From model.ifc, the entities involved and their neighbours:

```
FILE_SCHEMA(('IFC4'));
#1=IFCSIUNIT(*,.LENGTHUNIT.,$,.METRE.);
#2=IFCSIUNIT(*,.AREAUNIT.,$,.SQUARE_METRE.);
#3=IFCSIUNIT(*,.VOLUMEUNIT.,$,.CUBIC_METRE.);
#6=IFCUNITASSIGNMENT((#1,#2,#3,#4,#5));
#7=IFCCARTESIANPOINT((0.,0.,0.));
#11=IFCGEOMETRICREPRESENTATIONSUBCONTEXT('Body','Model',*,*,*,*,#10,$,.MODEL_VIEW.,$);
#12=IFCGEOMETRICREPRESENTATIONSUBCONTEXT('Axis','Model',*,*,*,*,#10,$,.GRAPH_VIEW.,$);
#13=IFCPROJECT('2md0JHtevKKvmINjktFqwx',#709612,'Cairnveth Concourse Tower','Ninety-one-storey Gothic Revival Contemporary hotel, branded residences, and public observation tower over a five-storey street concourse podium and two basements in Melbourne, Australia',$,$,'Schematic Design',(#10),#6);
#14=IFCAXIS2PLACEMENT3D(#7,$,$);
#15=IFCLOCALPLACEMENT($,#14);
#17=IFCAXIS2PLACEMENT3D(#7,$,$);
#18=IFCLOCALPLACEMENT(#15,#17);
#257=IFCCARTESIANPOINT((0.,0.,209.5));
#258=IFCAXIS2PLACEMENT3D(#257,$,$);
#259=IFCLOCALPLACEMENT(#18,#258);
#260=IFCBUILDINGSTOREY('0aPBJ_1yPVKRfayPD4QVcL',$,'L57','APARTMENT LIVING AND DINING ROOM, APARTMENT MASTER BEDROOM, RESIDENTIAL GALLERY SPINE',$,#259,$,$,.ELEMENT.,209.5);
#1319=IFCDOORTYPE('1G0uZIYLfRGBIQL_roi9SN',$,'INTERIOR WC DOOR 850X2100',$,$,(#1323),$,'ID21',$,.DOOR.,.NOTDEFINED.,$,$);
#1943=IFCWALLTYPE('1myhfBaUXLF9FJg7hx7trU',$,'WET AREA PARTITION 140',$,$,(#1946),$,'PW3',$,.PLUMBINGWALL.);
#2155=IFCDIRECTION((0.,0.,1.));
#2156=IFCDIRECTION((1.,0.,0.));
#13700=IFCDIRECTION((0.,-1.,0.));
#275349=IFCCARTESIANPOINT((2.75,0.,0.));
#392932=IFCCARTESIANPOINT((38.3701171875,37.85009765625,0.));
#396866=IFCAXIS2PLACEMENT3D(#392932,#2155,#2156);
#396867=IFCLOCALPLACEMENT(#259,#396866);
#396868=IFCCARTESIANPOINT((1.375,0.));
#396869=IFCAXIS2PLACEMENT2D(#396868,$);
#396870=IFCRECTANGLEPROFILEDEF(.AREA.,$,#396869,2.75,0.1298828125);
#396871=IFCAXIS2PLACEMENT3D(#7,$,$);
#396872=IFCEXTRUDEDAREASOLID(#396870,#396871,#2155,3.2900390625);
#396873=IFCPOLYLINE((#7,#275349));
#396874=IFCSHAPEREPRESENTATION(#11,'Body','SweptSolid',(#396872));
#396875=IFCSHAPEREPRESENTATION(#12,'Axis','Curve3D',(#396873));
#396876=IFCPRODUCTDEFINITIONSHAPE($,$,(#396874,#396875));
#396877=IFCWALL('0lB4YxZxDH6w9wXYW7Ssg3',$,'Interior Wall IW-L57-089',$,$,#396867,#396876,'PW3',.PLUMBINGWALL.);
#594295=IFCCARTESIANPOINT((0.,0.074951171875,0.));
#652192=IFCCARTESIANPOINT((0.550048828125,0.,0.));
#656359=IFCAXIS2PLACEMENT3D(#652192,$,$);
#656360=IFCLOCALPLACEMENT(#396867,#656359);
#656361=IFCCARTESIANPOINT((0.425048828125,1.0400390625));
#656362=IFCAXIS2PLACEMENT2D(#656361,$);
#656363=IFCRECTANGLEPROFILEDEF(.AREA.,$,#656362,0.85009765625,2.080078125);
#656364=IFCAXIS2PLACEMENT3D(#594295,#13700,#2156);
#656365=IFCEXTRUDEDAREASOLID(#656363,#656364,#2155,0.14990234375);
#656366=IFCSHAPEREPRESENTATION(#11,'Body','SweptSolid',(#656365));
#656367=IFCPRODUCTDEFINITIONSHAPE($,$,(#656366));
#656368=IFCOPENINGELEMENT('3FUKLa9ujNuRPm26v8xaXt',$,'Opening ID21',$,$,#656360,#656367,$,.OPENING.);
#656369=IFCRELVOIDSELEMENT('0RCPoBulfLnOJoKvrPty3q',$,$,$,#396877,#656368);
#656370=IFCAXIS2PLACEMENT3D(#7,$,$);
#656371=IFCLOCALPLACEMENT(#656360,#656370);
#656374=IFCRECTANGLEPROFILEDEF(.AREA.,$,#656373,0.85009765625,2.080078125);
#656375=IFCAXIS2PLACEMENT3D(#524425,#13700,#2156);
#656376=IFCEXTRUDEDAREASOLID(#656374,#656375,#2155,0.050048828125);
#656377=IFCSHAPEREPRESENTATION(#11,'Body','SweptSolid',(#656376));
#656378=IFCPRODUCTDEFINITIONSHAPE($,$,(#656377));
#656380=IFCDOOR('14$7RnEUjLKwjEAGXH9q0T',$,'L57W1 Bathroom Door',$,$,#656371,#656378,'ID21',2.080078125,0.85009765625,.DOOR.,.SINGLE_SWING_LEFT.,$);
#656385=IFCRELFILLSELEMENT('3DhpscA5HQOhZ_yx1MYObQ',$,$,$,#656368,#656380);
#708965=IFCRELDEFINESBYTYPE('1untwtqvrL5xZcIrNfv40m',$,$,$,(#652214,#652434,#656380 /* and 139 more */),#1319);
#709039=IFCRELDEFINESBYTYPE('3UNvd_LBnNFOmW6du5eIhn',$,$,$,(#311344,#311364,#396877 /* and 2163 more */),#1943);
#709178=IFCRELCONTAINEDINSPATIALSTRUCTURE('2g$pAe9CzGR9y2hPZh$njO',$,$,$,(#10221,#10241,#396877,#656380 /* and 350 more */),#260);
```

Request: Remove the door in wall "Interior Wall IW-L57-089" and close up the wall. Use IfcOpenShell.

```python
import ifcopenshell
import ifcopenshell.api.feature
import ifcopenshell.api.root
import ifcopenshell.geom
import ifcopenshell.util.shape

model = ifcopenshell.open("model.ifc")
settings = ifcopenshell.geom.settings()


def volume(element):
    """Net volume in cubic metres, openings subtracted."""
    shape = ifcopenshell.geom.create_shape(settings, element)
    return ifcopenshell.util.shape.get_volume(shape.geometry)


door = model.by_id(656380)
opening = door.FillsVoids[0].RelatingOpeningElement
wall = opening.VoidsElements[0].RelatingBuildingElement
before = volume(wall)

ifcopenshell.api.root.remove_product(model, product=door)
ifcopenshell.api.feature.remove_feature(model, feature=opening)

after = volume(wall)

print(f"wall volume {before:.3f} -> {after:.3f} m3")

model.write("model-out.ifc")
```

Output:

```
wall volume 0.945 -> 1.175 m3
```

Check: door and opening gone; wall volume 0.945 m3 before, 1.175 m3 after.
